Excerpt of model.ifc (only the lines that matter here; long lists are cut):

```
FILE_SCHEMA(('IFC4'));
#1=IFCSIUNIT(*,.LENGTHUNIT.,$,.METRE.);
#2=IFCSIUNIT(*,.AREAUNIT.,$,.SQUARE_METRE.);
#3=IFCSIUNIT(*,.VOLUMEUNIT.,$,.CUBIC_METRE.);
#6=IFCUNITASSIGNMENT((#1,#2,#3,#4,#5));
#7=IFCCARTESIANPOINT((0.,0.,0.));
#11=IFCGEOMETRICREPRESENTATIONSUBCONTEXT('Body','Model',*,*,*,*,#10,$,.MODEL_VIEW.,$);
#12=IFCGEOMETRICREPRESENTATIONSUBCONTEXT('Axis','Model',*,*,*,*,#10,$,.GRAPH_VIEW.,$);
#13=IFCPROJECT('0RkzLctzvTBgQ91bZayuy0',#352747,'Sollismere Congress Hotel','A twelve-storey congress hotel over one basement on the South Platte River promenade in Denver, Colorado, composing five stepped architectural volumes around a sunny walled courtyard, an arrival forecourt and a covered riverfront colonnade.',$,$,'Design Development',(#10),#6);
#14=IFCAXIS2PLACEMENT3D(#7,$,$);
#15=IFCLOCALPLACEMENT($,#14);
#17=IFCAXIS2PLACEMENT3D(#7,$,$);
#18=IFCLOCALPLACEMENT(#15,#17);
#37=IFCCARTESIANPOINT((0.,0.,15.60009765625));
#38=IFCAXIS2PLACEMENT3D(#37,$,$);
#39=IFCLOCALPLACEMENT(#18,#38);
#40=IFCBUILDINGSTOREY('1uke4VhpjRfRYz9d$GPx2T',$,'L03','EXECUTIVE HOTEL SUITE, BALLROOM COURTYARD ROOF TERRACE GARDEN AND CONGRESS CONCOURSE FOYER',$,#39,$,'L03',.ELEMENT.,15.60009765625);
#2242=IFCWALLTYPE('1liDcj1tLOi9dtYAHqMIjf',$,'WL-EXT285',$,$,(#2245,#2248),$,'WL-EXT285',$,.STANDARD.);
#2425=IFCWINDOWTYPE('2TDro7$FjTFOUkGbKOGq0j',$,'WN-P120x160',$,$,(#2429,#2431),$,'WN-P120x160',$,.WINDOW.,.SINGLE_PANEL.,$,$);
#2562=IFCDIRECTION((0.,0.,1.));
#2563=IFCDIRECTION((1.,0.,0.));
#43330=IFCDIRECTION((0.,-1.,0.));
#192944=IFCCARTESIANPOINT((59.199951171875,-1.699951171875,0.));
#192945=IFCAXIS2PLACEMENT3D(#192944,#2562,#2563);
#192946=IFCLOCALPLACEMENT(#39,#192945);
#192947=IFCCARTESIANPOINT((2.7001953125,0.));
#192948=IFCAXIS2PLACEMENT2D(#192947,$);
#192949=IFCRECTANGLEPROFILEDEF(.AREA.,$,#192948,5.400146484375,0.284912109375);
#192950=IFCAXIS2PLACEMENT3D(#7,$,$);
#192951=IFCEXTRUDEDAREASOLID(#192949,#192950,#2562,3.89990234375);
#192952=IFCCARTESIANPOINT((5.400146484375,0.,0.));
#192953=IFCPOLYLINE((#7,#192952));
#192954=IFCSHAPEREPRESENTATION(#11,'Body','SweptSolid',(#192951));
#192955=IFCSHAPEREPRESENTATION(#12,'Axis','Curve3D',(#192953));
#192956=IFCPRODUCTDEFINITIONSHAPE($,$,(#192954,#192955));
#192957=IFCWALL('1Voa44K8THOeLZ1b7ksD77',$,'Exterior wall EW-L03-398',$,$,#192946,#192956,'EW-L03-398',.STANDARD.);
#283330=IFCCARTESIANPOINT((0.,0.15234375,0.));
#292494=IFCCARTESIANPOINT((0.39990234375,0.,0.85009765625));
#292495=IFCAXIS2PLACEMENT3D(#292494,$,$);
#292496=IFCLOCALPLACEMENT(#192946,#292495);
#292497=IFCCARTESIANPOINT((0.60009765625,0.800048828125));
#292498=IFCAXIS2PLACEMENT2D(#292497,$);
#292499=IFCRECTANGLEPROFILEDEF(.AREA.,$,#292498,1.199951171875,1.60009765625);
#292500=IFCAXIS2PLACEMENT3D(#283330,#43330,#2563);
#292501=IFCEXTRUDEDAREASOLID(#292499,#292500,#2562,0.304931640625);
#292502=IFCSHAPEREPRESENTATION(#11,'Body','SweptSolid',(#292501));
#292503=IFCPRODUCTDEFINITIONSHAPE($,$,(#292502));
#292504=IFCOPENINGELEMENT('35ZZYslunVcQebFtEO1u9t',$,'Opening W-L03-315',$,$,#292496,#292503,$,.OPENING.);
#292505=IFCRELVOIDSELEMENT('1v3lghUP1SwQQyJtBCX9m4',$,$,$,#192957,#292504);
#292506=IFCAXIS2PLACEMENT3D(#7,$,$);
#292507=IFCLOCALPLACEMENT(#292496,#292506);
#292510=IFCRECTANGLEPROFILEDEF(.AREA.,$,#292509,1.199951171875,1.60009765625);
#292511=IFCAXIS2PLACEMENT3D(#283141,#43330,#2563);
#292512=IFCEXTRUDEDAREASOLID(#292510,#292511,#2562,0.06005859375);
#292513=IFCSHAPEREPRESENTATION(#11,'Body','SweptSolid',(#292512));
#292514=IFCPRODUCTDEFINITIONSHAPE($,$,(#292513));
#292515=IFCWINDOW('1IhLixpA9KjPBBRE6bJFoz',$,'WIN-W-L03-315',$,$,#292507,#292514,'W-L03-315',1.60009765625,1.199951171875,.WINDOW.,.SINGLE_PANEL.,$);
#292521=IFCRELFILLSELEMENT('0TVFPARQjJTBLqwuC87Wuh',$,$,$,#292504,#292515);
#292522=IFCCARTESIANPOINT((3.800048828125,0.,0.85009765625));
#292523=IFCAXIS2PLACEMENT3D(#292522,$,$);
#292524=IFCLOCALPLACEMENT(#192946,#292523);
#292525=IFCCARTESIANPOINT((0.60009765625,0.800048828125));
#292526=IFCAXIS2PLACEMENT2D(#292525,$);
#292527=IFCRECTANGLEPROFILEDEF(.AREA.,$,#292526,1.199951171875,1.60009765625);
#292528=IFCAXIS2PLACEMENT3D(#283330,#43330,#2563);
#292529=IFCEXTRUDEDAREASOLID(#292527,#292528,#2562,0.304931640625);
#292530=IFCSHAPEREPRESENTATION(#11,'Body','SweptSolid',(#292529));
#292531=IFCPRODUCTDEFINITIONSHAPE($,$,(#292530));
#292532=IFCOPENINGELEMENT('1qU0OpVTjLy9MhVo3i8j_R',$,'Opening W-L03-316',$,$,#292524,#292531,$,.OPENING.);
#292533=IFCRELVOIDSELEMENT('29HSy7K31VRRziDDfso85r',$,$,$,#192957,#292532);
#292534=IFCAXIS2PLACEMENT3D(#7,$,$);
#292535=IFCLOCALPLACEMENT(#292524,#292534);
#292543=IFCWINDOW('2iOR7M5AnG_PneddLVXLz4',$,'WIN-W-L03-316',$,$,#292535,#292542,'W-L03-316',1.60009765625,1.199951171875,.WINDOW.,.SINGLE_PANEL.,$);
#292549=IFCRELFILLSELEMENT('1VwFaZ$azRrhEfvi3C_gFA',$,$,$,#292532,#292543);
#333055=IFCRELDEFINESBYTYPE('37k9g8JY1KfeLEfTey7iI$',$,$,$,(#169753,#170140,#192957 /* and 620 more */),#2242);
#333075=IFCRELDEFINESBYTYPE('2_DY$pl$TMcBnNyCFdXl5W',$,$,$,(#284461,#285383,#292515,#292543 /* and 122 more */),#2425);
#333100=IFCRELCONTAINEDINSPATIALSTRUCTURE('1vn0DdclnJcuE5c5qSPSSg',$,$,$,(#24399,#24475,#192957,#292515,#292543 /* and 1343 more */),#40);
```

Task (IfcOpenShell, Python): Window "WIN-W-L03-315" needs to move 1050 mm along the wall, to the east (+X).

```python
import ifcopenshell
import ifcopenshell.api.geometry
import ifcopenshell.util.placement

model = ifcopenshell.open("model.ifc")

window = model.by_guid("1IhLixpA9KjPBBRE6bJFoz")
opening = window.FillsVoids[0].RelatingOpeningElement
wall = opening.VoidsElements[0].RelatingBuildingElement

wall_matrix = ifcopenshell.util.placement.get_local_placement(wall.ObjectPlacement)
shift = wall_matrix[:3, 0] * 1.05
before = ifcopenshell.util.placement.get_local_placement(window.ObjectPlacement)[:3, 3].copy()

# The window is placed relative to its opening, so it follows when the opening moves.
matrix = ifcopenshell.util.placement.get_local_placement(opening.ObjectPlacement)
matrix[:3, 3] += shift
ifcopenshell.api.geometry.edit_object_placement(
    model, product=opening, matrix=matrix, is_si=False, should_transform_children=True
)

after = ifcopenshell.util.placement.get_local_placement(window.ObjectPlacement)[:3, 3]
print("window moved by", (after - before).round(3) + 0.0)

model.write("model_updated.ifc")
```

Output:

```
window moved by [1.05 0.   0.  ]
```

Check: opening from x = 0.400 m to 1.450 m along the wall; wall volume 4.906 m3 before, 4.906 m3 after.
